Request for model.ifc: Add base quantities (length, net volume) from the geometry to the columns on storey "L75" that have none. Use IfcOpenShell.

First a look at what the model holds.

```python
import ifcopenshell
import ifcopenshell.util.element
import ifcopenshell.util.unit

model = ifcopenshell.open("model.ifc")
print(model.schema)
for unit_type in ("LENGTHUNIT", "AREAUNIT", "VOLUMEUNIT"):
    print(unit_type, ifcopenshell.util.unit.calculate_unit_scale(model, unit_type))
storey = next(s for s in model.by_type("IfcBuildingStorey") if s.Name == "L75")
columns = [e for e in ifcopenshell.util.element.get_decomposition(storey) if e.is_a("IfcColumn")]
for e in sorted(columns, key=lambda e: e.id()):
    print(e.id(), e.is_a(), e.Name, list(ifcopenshell.util.element.get_psets(e, qtos_only=True)), sep=" | ")
```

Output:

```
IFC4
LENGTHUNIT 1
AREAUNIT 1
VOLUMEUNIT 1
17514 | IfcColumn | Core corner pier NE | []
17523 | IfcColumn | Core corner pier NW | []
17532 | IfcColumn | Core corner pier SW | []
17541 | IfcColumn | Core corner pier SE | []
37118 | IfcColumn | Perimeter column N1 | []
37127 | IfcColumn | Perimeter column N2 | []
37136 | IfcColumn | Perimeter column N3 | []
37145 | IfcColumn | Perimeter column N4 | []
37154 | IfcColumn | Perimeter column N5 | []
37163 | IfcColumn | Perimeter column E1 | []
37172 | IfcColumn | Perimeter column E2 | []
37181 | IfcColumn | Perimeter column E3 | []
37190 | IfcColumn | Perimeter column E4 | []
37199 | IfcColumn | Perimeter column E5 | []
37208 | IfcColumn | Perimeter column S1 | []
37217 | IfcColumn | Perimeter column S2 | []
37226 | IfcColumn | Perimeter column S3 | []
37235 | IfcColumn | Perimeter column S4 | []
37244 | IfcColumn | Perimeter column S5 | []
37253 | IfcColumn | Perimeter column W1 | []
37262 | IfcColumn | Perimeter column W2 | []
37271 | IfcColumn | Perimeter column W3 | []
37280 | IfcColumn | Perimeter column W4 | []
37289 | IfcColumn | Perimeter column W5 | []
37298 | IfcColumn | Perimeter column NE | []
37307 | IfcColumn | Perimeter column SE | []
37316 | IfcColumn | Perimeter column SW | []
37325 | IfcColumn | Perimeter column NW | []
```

```python
import ifcopenshell
import ifcopenshell.api.pset
import ifcopenshell.geom
import ifcopenshell.util.element
import ifcopenshell.util.shape
import ifcopenshell.util.unit

model = ifcopenshell.open("model.ifc")
unit_scale = ifcopenshell.util.unit.calculate_unit_scale(model)
volume_scale = ifcopenshell.util.unit.calculate_unit_scale(model, "VOLUMEUNIT")
settings = ifcopenshell.geom.settings()

storey = next(s for s in model.by_type("IfcBuildingStorey") if s.Name == "L75")
columns = [e for e in ifcopenshell.util.element.get_decomposition(storey) if e.is_a("IfcColumn")]

for e in sorted(columns, key=lambda e: e.id()):
    if ifcopenshell.util.element.get_psets(e, qtos_only=True, should_inherit=False):
        continue
    # Geometry comes back in metres, in the element's own axes.
    shape = ifcopenshell.geom.create_shape(settings, e)
    values = {
        "Length": ifcopenshell.util.shape.get_z(shape.geometry) / unit_scale,
        "NetVolume": ifcopenshell.util.shape.get_volume(shape.geometry) / volume_scale,
    }
    qto = ifcopenshell.api.pset.add_qto(model, product=e, name="Qto_ColumnBaseQuantities")
    ifcopenshell.api.pset.edit_qto(model, qto=qto, properties=values)
    print(e.id(), {k: round(v, 3) for k, v in values.items()})

model.write("model_updated.ifc")
```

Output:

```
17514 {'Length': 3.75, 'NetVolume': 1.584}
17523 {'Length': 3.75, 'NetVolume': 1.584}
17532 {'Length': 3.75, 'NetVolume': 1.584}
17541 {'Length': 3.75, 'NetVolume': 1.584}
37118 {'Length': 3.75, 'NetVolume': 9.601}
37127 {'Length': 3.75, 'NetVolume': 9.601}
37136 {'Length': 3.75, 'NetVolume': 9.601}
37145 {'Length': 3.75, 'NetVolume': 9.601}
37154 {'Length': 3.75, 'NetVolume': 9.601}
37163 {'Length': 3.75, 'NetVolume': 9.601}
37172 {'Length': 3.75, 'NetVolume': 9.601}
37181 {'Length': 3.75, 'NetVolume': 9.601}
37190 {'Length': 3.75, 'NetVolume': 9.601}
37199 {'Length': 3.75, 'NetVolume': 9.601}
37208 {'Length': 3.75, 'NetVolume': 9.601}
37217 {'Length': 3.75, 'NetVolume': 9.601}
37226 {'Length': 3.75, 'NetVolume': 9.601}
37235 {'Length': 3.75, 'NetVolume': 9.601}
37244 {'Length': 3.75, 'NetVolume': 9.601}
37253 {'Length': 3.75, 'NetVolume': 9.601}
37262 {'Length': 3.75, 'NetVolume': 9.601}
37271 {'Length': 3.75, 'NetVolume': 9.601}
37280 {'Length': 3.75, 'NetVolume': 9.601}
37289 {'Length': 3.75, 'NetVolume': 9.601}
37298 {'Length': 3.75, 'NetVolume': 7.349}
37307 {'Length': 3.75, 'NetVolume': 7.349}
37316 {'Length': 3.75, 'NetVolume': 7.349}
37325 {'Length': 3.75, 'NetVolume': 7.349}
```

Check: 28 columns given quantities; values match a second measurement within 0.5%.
